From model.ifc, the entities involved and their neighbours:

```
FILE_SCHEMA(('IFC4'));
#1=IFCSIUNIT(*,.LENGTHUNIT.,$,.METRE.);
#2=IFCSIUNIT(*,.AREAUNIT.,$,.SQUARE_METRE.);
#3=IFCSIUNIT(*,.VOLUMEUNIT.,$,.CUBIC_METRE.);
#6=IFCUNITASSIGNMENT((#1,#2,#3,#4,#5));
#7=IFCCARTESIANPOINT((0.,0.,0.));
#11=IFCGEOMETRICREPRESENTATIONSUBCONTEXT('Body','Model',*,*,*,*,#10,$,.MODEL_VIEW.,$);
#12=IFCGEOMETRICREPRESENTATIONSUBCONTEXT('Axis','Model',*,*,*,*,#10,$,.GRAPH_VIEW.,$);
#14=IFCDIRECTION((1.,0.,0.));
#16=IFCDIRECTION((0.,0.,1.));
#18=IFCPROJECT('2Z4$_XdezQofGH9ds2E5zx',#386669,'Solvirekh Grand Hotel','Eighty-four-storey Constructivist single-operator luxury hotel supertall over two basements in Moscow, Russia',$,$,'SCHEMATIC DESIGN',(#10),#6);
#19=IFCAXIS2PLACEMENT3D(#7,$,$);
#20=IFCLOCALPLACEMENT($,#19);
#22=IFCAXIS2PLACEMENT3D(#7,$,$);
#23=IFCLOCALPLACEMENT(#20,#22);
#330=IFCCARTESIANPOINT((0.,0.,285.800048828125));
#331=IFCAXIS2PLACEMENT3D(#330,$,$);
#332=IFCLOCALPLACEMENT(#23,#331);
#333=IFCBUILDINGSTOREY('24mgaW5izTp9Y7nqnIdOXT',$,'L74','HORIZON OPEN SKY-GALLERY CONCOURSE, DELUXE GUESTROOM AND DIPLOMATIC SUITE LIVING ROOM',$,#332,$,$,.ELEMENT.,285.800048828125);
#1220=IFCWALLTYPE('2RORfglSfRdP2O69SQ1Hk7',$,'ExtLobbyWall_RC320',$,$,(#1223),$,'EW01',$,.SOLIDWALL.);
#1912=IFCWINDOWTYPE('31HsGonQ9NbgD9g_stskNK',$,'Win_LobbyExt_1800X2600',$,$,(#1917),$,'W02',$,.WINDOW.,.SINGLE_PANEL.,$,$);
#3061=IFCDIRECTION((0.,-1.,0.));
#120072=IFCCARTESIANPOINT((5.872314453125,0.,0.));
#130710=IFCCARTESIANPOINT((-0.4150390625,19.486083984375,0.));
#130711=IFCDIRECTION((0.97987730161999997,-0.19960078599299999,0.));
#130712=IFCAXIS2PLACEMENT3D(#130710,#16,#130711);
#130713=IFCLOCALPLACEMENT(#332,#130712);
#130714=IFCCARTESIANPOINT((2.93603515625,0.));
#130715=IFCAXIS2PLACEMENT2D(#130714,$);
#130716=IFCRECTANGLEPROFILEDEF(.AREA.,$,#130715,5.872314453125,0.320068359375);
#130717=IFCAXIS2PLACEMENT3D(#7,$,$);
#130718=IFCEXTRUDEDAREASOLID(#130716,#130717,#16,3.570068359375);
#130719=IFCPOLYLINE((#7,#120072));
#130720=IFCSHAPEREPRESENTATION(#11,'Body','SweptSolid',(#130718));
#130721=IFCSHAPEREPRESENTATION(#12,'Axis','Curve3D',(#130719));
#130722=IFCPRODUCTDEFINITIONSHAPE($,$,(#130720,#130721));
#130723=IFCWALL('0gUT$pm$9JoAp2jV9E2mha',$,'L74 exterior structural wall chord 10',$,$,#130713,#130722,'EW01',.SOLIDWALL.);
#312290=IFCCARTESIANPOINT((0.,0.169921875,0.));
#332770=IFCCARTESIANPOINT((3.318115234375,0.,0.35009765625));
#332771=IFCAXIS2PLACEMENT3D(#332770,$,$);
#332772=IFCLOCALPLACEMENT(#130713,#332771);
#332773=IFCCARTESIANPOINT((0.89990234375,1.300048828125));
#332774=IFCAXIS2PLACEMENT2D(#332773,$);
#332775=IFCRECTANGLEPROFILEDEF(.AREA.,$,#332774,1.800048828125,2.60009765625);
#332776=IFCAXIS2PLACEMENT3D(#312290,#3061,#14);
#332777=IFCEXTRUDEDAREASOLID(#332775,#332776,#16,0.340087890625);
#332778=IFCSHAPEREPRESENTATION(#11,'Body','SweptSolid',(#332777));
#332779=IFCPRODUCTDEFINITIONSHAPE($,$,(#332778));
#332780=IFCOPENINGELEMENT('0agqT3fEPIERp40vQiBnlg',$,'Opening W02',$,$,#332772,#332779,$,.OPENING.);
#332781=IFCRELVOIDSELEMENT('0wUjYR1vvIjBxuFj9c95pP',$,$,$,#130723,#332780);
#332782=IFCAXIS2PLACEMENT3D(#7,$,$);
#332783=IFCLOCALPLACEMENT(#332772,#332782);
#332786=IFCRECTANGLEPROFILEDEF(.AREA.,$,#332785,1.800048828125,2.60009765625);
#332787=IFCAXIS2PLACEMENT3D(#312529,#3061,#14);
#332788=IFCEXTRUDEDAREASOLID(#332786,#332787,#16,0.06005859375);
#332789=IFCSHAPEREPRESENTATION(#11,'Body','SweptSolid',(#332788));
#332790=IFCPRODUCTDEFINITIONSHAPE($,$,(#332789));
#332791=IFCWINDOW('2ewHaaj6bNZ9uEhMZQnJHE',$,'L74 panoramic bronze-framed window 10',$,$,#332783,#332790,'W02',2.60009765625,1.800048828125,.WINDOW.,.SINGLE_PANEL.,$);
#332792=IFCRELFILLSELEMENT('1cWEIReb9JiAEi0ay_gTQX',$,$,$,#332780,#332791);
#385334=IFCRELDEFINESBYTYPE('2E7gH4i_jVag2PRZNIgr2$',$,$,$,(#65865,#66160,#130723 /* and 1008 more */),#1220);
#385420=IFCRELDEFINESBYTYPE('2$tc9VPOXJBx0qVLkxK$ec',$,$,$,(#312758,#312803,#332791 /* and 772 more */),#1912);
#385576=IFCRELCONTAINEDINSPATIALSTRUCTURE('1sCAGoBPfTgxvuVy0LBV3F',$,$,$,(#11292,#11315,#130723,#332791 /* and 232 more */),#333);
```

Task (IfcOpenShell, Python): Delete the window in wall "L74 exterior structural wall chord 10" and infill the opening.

```python
import ifcopenshell
import ifcopenshell.api.feature
import ifcopenshell.api.root
import ifcopenshell.geom
import ifcopenshell.util.shape

model = ifcopenshell.open("model.ifc")
settings = ifcopenshell.geom.settings()


def volume(element):
    """Net volume in cubic metres, openings subtracted."""
    shape = ifcopenshell.geom.create_shape(settings, element)
    return ifcopenshell.util.shape.get_volume(shape.geometry)


window = model.by_guid("2ewHaaj6bNZ9uEhMZQnJHE")
opening = window.FillsVoids[0].RelatingOpeningElement
wall = opening.VoidsElements[0].RelatingBuildingElement
before = volume(wall)

ifcopenshell.api.root.remove_product(model, product=window)
ifcopenshell.api.feature.remove_feature(model, feature=opening)

after = volume(wall)

print(f"wall volume {before:.3f} -> {after:.3f} m3")

model.write("model_v2.ifc")
```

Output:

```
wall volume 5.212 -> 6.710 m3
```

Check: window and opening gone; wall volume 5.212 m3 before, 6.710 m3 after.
